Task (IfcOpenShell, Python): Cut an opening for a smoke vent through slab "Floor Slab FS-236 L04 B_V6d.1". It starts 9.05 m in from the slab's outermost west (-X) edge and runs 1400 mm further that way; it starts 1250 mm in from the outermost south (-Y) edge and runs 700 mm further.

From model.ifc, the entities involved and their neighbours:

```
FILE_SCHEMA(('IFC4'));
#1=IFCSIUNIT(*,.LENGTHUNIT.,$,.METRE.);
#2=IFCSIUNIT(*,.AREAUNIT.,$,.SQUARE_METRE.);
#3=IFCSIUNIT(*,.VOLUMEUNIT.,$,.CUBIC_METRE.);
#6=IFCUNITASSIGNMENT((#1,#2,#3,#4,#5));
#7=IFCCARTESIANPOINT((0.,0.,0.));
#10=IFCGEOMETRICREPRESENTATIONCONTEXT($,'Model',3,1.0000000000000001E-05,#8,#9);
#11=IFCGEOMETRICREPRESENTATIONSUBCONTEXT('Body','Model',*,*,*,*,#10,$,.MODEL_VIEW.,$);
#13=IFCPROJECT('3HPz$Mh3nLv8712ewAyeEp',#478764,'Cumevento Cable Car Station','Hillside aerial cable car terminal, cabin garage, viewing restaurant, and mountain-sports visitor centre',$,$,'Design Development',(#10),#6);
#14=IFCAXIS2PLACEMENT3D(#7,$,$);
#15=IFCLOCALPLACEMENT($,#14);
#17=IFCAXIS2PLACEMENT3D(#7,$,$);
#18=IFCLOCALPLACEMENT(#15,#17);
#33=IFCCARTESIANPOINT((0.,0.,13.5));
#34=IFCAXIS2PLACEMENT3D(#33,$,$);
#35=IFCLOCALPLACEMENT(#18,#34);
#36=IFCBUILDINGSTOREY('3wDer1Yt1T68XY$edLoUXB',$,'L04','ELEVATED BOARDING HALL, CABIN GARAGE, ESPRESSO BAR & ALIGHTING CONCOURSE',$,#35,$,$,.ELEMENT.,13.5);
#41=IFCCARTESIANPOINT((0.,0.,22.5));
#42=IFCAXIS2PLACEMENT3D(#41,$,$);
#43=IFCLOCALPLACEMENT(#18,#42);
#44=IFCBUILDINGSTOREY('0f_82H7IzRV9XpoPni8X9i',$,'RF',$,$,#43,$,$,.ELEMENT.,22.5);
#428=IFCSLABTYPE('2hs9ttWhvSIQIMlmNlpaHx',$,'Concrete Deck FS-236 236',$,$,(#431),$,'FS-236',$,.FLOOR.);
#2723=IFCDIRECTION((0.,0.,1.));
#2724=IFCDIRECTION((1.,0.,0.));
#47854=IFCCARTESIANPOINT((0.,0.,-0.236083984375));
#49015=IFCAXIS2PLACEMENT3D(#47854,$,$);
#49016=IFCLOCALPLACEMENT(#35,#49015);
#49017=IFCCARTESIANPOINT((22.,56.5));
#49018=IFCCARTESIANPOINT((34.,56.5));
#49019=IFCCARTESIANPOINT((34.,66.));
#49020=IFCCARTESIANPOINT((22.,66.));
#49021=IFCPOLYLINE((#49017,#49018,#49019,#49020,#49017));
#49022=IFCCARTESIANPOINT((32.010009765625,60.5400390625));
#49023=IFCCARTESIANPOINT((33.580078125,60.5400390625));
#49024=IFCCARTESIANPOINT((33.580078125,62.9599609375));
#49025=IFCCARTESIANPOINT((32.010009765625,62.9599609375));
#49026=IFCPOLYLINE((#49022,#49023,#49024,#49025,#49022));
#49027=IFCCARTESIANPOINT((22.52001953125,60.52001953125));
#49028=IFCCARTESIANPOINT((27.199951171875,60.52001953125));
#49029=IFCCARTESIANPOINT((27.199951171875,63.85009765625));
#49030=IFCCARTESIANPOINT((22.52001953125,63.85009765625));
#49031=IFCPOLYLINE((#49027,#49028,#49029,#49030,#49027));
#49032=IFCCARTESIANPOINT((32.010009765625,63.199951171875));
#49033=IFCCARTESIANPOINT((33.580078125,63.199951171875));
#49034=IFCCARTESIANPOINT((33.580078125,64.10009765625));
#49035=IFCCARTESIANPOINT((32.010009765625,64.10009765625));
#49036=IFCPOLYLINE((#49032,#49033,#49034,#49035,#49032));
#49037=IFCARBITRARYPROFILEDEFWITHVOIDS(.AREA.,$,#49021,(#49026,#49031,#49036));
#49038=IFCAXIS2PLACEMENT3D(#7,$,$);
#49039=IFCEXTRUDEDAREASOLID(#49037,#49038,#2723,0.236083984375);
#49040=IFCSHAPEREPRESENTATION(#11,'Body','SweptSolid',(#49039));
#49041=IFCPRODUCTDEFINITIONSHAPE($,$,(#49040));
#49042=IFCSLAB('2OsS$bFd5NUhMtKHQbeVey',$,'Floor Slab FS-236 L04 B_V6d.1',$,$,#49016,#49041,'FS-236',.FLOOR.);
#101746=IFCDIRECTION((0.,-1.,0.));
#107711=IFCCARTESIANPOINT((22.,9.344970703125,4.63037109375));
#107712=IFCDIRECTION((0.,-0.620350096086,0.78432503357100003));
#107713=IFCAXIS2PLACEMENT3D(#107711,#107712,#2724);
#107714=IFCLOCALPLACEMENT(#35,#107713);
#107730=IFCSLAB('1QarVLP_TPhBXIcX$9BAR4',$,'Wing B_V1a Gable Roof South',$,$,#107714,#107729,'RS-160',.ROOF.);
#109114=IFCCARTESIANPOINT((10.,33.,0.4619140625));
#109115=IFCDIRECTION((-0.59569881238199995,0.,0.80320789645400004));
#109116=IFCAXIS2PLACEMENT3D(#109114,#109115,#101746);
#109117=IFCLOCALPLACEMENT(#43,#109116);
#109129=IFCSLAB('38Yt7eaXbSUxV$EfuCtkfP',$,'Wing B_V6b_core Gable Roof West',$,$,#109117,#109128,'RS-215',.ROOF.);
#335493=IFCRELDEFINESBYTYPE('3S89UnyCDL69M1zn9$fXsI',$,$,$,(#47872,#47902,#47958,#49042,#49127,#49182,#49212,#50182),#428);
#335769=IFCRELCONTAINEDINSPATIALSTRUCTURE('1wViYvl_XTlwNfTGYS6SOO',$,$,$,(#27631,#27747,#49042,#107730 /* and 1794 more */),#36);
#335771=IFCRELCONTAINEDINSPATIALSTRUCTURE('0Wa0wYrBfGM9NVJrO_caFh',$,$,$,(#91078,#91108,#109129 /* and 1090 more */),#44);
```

```python
import numpy as np
import ifcopenshell
import ifcopenshell.api.feature
import ifcopenshell.api.geometry
import ifcopenshell.api.root
import ifcopenshell.geom
import ifcopenshell.util.placement
import ifcopenshell.util.representation
import ifcopenshell.util.shape
import ifcopenshell.util.unit

model = ifcopenshell.open("model.ifc")
unit_scale = ifcopenshell.util.unit.calculate_unit_scale(model)
settings = ifcopenshell.geom.settings()


def volume(element):
    """Net volume in cubic metres, openings subtracted."""
    shape = ifcopenshell.geom.create_shape(settings, element)
    return ifcopenshell.util.shape.get_volume(shape.geometry)


slab = model.by_id(49042)
before = volume(slab)

# Extent in the slab's own axes, in metres. The edges named are its -X and -Y sides.
slab_shape = ifcopenshell.geom.create_shape(settings, slab)
vertices = ifcopenshell.util.shape.get_vertices(slab_shape.geometry)
x_min, y_min, bottom = vertices.min(axis=0)
top = vertices[:, 2].max()

opening = ifcopenshell.api.root.create_entity(model, ifc_class="IfcOpeningElement", name="Smoke vent opening", predefined_type="OPENING")
context = ifcopenshell.util.representation.get_context(model, "Model", "Body", "MODEL_VIEW")
width, depth = 1.4, 0.7
outline = [(0.0, 0.0), (width, 0.0), (width, depth), (0.0, depth), (0.0, 0.0)]
# Overshoot both faces by 50 mm so the cut is clean.
shape = ifcopenshell.api.geometry.add_slab_representation(
    model, context=context, depth=top - bottom + 0.1, polyline=outline
)
ifcopenshell.api.geometry.assign_representation(model, product=opening, representation=shape)

matrix = ifcopenshell.util.placement.get_local_placement(slab.ObjectPlacement)
matrix[:, 3] = matrix @ np.append(np.array([x_min + 9.05, y_min + 1.25, bottom - 0.05]) / unit_scale, 1.0)
ifcopenshell.api.geometry.edit_object_placement(model, product=opening, matrix=matrix, is_si=False)
ifcopenshell.api.feature.add_feature(model, feature=opening, element=slab)

after = volume(slab)

print(f"slab volume {before:.3f} -> {after:.3f} m3")

model.write("model_rev.ifc")
```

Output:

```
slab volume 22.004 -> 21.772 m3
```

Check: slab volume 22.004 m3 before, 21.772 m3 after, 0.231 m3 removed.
